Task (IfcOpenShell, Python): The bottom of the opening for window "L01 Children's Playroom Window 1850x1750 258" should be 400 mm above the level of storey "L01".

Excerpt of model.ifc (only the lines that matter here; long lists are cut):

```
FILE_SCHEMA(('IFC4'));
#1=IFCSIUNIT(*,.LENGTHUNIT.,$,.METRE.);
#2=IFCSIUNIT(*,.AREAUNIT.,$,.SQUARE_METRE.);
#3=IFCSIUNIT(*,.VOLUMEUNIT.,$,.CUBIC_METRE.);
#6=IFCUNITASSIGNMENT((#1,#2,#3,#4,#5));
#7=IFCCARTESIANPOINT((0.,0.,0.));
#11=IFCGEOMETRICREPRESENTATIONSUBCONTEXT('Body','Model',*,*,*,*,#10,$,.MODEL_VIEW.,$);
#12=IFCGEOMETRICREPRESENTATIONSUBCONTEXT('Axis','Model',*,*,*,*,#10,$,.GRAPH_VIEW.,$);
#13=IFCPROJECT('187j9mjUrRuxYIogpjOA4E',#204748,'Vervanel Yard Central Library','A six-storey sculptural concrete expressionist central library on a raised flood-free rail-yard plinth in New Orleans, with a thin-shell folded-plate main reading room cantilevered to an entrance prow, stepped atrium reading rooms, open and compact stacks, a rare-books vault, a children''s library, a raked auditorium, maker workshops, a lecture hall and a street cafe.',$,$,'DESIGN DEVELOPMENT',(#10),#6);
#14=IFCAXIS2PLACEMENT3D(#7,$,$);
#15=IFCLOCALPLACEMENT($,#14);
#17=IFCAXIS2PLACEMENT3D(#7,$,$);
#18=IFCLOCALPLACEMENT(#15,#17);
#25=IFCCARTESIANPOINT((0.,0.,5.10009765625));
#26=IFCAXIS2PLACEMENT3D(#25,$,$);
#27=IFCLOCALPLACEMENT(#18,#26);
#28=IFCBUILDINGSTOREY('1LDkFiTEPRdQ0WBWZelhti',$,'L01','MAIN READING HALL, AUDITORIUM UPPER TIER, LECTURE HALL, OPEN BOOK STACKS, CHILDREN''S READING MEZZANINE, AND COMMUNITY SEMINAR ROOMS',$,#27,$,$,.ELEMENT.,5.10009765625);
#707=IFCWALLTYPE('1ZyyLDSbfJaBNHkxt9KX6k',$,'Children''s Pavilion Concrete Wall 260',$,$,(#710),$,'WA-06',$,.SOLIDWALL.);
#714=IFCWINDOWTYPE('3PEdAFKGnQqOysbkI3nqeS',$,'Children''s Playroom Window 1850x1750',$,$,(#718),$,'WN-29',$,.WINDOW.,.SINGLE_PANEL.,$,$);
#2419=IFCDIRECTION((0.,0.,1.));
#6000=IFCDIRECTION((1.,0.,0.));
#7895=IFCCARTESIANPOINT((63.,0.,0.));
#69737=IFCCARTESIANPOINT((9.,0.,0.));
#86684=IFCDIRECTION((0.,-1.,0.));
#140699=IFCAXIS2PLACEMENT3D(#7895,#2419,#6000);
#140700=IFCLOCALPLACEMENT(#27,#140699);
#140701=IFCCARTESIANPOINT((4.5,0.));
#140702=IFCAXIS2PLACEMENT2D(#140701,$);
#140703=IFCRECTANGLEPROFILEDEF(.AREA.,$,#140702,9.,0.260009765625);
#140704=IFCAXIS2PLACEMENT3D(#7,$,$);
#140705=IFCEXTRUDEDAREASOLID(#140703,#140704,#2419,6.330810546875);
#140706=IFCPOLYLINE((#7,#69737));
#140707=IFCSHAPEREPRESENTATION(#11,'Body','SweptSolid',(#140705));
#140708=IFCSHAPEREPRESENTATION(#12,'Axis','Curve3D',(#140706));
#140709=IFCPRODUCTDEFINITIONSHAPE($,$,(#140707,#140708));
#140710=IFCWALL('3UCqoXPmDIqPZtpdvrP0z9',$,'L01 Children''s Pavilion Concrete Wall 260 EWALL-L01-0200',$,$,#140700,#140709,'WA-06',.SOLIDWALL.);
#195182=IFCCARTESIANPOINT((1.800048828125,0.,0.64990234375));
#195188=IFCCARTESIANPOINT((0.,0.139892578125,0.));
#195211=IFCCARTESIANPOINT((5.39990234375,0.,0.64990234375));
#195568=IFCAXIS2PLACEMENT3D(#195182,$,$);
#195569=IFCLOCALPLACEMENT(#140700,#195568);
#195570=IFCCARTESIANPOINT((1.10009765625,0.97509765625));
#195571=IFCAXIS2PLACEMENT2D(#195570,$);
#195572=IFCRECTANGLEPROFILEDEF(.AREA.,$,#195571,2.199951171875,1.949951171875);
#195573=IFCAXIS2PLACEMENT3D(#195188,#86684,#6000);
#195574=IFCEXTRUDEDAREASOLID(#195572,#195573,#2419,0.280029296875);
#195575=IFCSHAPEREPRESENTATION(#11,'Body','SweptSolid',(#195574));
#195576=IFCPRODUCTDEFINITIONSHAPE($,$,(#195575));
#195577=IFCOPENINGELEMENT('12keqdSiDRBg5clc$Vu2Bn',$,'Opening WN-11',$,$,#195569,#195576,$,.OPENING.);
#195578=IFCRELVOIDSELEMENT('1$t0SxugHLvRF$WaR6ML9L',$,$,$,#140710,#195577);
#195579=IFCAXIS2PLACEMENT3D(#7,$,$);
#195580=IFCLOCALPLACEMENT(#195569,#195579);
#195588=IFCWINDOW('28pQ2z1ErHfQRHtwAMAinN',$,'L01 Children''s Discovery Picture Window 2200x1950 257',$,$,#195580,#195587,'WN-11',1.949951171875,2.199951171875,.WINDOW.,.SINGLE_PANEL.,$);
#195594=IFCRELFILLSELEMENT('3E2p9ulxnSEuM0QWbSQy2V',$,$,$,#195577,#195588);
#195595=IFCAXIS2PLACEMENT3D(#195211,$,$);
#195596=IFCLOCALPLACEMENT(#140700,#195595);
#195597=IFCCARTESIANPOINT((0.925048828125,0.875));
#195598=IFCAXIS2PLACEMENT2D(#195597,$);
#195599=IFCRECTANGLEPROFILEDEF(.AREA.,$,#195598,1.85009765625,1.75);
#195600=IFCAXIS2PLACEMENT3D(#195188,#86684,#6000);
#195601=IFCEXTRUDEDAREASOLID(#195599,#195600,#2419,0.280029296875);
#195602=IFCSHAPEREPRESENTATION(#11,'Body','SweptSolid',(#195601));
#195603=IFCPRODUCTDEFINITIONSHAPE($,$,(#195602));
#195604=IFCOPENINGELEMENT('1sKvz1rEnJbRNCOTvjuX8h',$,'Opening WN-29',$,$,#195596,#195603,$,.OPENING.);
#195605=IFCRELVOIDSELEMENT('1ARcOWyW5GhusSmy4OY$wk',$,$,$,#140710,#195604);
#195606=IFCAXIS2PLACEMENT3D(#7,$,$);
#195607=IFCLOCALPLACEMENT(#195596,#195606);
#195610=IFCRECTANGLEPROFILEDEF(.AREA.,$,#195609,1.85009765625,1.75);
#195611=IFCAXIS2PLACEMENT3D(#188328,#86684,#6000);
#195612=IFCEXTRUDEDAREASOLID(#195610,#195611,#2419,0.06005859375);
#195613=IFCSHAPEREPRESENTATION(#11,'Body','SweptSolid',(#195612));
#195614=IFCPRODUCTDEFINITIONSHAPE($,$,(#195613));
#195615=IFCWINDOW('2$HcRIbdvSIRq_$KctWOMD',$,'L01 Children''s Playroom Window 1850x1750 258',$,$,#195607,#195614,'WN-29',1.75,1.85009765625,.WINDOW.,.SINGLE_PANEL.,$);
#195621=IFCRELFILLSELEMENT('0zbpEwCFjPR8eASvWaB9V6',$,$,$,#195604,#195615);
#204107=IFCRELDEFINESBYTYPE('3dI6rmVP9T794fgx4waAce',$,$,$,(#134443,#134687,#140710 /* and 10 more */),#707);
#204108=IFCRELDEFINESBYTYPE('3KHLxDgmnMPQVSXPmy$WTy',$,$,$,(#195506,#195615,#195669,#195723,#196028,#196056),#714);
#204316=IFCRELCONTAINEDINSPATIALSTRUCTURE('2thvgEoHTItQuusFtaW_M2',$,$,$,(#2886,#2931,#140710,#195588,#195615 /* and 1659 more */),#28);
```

```python
import numpy as np
import ifcopenshell
import ifcopenshell.api.geometry
import ifcopenshell.geom
import ifcopenshell.util.element
import ifcopenshell.util.placement
import ifcopenshell.util.shape
import ifcopenshell.util.unit

model = ifcopenshell.open("model.ifc")
unit_scale = ifcopenshell.util.unit.calculate_unit_scale(model)

window = model.by_id(195615)
opening = window.FillsVoids[0].RelatingOpeningElement
storey = ifcopenshell.util.element.get_container(window, ifc_class="IfcBuildingStorey")
level = ifcopenshell.util.placement.get_local_placement(storey.ObjectPlacement)[2, 3]

# The opening's origin need not be at the sill, so measure its lowest point.
shape = ifcopenshell.geom.create_shape(ifcopenshell.geom.settings(), opening)
bottom = ifcopenshell.util.shape.get_shape_bottom_elevation(shape, shape.geometry) / unit_scale
dz = level + 0.4 - bottom

shift = np.array([0.0, 0.0, dz])
# The window is placed relative to its opening, so it follows when the opening moves.
matrix = ifcopenshell.util.placement.get_local_placement(opening.ObjectPlacement)
matrix[:3, 3] += shift
ifcopenshell.api.geometry.edit_object_placement(
    model, product=opening, matrix=matrix, is_si=False, should_transform_children=True
)

print(f"moved by {dz * unit_scale:+.3f} m")

model.write("model_rev.ifc")
```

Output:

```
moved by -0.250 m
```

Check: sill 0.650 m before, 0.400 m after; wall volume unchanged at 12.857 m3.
